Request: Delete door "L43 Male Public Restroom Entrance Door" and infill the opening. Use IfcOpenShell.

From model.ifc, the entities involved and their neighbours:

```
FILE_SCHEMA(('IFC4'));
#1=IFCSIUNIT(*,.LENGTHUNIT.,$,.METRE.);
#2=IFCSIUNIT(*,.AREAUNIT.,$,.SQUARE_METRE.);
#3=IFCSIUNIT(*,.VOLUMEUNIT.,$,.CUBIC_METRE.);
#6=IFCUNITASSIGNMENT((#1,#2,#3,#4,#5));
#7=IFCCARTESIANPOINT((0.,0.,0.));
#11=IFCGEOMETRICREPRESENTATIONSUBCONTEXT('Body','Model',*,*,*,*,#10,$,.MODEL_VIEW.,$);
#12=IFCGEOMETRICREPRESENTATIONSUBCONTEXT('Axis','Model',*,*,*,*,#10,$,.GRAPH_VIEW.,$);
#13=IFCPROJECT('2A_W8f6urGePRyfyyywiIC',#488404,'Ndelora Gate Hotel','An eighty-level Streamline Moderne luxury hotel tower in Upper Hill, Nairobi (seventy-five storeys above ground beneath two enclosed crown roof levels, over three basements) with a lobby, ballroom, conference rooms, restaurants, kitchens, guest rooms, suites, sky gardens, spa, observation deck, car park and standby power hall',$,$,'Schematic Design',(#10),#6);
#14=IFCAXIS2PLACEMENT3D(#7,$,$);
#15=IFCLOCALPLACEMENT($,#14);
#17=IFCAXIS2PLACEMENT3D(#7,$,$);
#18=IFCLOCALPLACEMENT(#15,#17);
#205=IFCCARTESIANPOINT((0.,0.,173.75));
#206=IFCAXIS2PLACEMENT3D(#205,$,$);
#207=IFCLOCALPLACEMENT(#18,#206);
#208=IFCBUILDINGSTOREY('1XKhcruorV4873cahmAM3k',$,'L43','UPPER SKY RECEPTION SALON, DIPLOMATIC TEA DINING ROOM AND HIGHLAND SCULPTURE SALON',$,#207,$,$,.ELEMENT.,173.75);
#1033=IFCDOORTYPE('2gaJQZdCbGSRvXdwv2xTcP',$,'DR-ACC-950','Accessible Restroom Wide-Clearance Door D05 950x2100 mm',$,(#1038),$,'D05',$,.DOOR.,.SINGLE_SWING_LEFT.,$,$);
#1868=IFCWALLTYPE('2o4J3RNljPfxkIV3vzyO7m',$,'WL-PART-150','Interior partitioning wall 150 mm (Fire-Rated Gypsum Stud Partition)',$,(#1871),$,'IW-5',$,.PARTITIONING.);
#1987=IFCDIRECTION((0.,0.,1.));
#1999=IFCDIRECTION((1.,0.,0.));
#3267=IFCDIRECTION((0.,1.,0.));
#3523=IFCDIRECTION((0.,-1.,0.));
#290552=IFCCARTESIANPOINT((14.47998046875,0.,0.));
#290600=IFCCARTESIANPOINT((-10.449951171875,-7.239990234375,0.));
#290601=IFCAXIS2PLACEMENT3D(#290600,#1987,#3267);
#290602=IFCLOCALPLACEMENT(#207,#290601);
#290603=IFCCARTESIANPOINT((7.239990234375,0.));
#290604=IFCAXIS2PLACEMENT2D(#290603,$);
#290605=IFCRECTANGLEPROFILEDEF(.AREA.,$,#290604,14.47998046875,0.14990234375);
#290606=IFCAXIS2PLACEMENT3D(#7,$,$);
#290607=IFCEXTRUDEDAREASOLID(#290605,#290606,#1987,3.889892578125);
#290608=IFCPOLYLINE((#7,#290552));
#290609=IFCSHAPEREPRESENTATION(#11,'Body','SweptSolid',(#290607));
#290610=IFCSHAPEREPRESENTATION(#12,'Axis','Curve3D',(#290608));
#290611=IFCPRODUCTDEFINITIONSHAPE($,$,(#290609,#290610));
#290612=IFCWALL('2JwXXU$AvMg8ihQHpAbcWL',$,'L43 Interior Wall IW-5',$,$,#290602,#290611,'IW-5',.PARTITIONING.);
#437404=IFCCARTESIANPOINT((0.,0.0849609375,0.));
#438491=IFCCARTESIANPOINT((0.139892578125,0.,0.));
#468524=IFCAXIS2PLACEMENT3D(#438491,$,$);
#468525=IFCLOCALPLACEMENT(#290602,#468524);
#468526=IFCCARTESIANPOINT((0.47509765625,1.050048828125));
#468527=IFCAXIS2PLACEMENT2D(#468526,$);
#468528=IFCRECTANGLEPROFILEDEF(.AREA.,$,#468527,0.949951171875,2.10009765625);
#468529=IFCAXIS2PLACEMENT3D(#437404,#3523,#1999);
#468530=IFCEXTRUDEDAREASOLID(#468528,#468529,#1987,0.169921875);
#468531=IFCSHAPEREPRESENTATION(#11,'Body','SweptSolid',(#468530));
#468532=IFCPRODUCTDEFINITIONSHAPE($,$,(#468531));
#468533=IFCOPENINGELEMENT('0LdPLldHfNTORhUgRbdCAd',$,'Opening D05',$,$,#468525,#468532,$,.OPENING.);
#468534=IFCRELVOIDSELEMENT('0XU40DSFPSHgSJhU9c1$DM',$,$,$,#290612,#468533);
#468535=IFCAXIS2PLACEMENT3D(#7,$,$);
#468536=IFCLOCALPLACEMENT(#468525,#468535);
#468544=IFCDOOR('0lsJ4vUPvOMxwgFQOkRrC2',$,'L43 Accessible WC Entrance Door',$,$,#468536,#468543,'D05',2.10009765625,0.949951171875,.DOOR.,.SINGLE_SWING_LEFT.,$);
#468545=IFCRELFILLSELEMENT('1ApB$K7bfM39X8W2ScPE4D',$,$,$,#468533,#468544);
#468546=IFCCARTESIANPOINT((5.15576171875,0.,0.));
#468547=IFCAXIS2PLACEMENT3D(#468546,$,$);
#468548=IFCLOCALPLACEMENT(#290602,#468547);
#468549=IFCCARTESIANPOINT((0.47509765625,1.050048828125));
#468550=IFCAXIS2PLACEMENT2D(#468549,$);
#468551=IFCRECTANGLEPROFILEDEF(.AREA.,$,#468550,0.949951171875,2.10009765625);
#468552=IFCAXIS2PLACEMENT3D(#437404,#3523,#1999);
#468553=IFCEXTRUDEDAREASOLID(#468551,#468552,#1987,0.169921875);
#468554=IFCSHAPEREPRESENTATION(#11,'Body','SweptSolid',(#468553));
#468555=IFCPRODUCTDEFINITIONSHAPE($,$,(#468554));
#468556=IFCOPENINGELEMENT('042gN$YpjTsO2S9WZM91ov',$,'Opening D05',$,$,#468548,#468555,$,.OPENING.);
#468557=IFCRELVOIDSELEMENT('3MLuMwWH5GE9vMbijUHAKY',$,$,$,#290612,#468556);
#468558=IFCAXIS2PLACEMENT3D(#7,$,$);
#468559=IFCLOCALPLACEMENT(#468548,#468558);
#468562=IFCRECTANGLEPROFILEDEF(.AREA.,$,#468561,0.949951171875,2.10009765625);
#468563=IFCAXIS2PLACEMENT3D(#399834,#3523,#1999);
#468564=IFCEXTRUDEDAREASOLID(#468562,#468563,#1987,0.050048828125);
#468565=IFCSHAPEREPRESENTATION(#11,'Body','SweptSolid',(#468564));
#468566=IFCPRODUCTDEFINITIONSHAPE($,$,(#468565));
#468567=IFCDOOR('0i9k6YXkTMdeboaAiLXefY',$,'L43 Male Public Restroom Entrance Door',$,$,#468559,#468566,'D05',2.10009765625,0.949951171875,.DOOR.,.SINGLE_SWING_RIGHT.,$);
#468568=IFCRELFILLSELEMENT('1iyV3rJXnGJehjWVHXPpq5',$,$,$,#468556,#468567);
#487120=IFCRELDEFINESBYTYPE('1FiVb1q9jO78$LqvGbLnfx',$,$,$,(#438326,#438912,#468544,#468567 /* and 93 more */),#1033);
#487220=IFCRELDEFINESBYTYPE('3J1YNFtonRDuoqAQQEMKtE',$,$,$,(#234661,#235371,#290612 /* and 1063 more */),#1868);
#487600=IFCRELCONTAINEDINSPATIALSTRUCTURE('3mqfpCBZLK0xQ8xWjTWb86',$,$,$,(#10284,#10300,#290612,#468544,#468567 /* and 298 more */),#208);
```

```python
import ifcopenshell
import ifcopenshell.api.feature
import ifcopenshell.api.root
import ifcopenshell.geom
import ifcopenshell.util.shape

model = ifcopenshell.open("model.ifc")
settings = ifcopenshell.geom.settings()


def volume(element):
    """Net volume in cubic metres, openings subtracted."""
    shape = ifcopenshell.geom.create_shape(settings, element)
    return ifcopenshell.util.shape.get_volume(shape.geometry)


door = model.by_guid("0i9k6YXkTMdeboaAiLXefY")
opening = door.FillsVoids[0].RelatingOpeningElement
wall = opening.VoidsElements[0].RelatingBuildingElement
before = volume(wall)

ifcopenshell.api.root.remove_product(model, product=door)
ifcopenshell.api.feature.remove_feature(model, feature=opening)

after = volume(wall)

print(f"wall volume {before:.3f} -> {after:.3f} m3")

model.write("model_v2.ifc")
```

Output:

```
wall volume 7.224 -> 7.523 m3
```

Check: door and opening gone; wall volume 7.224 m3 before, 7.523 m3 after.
